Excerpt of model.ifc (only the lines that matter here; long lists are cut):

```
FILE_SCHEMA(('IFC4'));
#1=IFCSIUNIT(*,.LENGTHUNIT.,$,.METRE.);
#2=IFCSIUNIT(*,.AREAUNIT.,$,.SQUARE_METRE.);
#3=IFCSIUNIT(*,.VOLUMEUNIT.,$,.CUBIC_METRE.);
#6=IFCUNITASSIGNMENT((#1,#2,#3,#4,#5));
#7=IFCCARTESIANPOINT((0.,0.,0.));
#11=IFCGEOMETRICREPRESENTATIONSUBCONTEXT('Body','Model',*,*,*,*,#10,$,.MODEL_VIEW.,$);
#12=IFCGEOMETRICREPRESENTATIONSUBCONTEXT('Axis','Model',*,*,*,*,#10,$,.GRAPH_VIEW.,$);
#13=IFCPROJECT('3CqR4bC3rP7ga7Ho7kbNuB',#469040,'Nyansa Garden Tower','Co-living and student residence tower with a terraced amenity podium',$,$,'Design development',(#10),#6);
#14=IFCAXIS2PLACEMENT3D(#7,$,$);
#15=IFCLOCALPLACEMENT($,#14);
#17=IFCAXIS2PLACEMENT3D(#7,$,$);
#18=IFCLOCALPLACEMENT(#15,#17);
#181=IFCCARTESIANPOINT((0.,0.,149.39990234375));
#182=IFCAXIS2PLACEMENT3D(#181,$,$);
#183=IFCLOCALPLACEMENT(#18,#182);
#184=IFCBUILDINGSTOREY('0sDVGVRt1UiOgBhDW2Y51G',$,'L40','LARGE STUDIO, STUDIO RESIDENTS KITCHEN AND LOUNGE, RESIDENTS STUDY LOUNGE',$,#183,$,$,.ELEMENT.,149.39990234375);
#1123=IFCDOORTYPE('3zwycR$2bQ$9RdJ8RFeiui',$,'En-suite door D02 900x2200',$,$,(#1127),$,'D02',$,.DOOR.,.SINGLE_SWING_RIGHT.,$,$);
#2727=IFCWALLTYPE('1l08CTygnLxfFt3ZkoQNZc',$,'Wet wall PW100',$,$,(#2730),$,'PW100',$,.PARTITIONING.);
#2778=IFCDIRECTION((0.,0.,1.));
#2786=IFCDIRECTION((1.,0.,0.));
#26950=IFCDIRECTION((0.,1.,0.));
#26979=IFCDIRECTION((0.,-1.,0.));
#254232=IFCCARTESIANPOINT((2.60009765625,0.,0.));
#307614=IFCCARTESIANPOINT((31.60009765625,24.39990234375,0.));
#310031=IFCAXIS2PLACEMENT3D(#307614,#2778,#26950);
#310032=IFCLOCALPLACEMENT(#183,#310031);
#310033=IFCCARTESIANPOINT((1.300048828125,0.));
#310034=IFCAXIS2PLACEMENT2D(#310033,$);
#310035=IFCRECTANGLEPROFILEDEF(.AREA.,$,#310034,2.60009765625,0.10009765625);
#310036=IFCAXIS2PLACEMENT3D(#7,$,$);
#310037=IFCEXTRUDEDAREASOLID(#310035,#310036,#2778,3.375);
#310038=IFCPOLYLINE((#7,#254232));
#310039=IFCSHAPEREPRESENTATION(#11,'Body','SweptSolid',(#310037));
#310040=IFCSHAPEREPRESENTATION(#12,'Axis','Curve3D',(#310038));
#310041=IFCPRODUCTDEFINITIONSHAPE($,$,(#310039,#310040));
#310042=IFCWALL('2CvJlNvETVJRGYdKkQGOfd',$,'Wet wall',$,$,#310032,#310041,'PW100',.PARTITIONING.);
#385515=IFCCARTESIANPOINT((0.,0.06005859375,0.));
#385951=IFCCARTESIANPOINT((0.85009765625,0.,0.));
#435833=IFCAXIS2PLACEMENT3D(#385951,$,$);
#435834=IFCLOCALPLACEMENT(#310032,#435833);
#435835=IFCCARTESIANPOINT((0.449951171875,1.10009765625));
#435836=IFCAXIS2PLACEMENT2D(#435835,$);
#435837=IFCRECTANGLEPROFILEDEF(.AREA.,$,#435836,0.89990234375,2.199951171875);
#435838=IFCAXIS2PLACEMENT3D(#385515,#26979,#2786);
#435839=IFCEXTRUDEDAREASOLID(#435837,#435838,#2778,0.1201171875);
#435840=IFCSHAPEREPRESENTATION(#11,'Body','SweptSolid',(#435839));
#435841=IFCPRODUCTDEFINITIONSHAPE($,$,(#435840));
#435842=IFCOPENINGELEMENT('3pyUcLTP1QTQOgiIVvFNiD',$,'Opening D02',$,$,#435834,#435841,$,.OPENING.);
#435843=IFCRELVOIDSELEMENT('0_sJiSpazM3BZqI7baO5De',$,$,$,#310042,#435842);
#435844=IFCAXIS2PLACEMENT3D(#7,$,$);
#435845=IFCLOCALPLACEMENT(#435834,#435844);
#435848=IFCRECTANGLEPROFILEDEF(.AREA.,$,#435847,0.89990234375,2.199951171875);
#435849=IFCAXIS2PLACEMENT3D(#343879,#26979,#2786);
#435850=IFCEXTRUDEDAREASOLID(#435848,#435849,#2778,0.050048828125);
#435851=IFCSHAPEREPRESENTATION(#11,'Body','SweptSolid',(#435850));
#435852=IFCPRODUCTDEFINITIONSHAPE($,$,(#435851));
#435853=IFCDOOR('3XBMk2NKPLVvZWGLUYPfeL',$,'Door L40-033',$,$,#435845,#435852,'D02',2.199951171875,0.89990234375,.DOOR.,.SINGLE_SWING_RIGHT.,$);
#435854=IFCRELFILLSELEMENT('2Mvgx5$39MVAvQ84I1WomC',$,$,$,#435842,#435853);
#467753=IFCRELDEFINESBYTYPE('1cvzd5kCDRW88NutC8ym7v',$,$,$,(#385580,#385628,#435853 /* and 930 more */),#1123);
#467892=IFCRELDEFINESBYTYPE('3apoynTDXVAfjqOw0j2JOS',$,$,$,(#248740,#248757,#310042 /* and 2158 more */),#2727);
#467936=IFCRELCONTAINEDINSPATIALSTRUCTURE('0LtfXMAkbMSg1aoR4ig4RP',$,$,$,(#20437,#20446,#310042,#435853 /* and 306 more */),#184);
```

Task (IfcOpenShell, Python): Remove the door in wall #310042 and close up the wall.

```python
import ifcopenshell
import ifcopenshell.api.feature
import ifcopenshell.api.root
import ifcopenshell.geom
import ifcopenshell.util.shape

model = ifcopenshell.open("model.ifc")
settings = ifcopenshell.geom.settings()


def volume(element):
    """Net volume in cubic metres, openings subtracted."""
    shape = ifcopenshell.geom.create_shape(settings, element)
    return ifcopenshell.util.shape.get_volume(shape.geometry)


door = model.by_guid("3XBMk2NKPLVvZWGLUYPfeL")
opening = door.FillsVoids[0].RelatingOpeningElement
wall = opening.VoidsElements[0].RelatingBuildingElement
before = volume(wall)

ifcopenshell.api.root.remove_product(model, product=door)
ifcopenshell.api.feature.remove_feature(model, feature=opening)

after = volume(wall)

print(f"wall volume {before:.3f} -> {after:.3f} m3")

model.write("model-out.ifc")
```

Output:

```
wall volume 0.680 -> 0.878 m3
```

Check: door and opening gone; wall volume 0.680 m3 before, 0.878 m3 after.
